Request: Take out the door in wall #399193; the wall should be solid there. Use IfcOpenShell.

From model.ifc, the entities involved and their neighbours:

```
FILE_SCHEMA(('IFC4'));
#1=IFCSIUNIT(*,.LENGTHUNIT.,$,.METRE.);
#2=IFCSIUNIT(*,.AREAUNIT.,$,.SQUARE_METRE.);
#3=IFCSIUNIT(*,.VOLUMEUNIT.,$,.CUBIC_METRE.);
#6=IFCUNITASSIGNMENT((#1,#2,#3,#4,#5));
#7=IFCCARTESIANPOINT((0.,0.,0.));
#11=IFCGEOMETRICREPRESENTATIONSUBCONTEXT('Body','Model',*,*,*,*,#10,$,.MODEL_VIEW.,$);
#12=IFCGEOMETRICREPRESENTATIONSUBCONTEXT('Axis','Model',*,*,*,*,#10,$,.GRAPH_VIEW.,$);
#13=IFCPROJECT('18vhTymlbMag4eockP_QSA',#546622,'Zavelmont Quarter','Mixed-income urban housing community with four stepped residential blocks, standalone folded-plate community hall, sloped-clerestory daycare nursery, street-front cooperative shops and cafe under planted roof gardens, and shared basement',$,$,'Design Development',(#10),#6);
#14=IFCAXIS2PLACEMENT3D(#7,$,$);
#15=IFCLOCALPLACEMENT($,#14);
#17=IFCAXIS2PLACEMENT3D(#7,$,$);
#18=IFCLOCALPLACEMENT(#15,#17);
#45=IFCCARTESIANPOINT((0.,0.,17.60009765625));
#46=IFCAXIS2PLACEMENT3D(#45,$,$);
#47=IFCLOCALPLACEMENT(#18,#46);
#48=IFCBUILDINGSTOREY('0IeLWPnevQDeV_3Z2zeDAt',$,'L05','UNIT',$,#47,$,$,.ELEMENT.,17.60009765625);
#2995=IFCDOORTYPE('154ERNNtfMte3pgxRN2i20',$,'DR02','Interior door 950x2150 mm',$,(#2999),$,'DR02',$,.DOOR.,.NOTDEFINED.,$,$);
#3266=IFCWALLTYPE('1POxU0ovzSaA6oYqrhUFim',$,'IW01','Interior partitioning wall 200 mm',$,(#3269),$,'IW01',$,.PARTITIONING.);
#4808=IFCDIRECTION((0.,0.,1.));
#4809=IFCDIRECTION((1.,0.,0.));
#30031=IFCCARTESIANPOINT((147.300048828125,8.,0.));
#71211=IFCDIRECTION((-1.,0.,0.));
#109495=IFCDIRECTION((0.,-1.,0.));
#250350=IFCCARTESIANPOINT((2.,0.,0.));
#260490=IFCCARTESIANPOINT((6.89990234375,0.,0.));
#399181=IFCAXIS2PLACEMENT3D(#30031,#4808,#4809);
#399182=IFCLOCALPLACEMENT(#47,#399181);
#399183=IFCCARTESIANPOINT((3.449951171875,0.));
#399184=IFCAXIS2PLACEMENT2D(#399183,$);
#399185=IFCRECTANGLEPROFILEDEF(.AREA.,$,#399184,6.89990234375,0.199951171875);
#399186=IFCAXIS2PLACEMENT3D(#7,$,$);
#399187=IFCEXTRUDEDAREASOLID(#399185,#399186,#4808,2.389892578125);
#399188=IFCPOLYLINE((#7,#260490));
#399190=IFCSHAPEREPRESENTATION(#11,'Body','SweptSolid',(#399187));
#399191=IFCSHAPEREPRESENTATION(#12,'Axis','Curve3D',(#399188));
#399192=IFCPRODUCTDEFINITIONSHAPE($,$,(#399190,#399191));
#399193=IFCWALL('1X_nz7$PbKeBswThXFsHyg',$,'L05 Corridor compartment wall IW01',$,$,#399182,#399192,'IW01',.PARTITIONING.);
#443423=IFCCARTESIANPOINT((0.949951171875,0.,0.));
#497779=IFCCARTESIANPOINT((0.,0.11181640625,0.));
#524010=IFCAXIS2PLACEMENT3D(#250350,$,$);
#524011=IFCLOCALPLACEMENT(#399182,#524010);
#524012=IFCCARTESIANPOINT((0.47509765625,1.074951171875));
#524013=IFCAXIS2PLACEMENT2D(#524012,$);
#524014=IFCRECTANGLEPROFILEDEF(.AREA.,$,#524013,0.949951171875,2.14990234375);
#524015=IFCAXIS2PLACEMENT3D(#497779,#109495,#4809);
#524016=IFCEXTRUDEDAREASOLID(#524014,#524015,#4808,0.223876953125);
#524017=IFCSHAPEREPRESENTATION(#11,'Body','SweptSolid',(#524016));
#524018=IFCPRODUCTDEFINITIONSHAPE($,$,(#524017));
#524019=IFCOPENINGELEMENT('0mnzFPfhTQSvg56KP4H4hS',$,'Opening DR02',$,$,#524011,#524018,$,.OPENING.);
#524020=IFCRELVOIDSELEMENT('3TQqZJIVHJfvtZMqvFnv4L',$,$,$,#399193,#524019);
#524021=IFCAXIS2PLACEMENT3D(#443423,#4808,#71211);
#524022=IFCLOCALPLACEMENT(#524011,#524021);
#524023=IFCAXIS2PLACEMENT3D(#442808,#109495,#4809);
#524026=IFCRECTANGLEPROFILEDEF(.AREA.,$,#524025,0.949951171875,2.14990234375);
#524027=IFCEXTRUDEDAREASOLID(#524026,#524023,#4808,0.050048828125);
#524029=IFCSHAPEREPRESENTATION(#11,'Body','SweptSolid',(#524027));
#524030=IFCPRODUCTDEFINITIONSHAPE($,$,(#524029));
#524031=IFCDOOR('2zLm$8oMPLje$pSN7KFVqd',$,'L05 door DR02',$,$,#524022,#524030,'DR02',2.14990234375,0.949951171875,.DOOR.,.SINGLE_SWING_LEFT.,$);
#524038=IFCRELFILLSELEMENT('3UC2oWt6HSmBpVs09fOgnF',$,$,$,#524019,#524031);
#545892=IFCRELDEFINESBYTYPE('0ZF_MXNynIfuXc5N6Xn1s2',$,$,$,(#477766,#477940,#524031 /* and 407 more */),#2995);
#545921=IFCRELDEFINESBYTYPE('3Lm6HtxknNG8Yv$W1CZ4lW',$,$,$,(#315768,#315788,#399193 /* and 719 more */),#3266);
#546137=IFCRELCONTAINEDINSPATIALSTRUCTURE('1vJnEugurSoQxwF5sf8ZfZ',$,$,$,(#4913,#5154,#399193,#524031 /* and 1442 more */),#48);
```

```python
import ifcopenshell
import ifcopenshell.api.feature
import ifcopenshell.api.root
import ifcopenshell.geom
import ifcopenshell.util.shape

model = ifcopenshell.open("model.ifc")
settings = ifcopenshell.geom.settings()


def volume(element):
    """Net volume in cubic metres, openings subtracted."""
    shape = ifcopenshell.geom.create_shape(settings, element)
    return ifcopenshell.util.shape.get_volume(shape.geometry)


door = model.by_guid("2zLm$8oMPLje$pSN7KFVqd")
opening = door.FillsVoids[0].RelatingOpeningElement
wall = opening.VoidsElements[0].RelatingBuildingElement
before = volume(wall)

ifcopenshell.api.root.remove_product(model, product=door)
ifcopenshell.api.feature.remove_feature(model, feature=opening)

after = volume(wall)

print(f"wall volume {before:.3f} -> {after:.3f} m3")

model.write("model_v2.ifc")
```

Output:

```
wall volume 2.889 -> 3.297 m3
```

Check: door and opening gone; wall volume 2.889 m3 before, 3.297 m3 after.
